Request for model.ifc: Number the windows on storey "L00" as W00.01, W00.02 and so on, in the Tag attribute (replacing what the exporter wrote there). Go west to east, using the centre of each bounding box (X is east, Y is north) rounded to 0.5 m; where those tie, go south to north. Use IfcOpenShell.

First a look at what the model holds.

```python
import ifcopenshell
import ifcopenshell.util.element
import ifcopenshell.util.placement

model = ifcopenshell.open("model.ifc")
print(model.schema)
storey = next(s for s in model.by_type("IfcBuildingStorey") if s.Name == "L00")
windows = [e for e in ifcopenshell.util.element.get_decomposition(storey) if e.is_a("IfcWindow")]
for e in sorted(windows, key=lambda e: e.id()):
    origin = ifcopenshell.util.placement.get_local_placement(e.ObjectPlacement)[:3, 3]
    print(e.id(), e.Tag, e.Name, origin.round(2) + 0.0, sep=" | ")
```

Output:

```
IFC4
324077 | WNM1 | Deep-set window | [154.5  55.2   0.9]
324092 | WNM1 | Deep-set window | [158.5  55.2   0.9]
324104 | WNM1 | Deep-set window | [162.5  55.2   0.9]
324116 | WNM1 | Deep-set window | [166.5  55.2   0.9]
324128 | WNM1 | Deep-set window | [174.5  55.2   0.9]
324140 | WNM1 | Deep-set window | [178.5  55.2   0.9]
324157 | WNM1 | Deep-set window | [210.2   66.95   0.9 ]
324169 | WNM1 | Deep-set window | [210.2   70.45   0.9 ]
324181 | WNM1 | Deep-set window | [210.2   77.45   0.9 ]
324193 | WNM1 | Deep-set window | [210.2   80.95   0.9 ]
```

```python
import ifcopenshell
import ifcopenshell.geom
import ifcopenshell.util.element
import ifcopenshell.util.shape

model = ifcopenshell.open("model.ifc")
settings = ifcopenshell.geom.settings()
settings.set("use-world-coords", True)


def centre(element):
    shape = ifcopenshell.geom.create_shape(settings, element)
    return ifcopenshell.util.shape.get_bbox_centroid(shape.geometry)


storey = next(s for s in model.by_type("IfcBuildingStorey") if s.Name == "L00")
windows = [e for e in ifcopenshell.util.element.get_decomposition(storey) if e.is_a("IfcWindow")]

# Insertion points can sit at a corner or the storey origin, so sort by the geometry (in metres).
centres = {e: centre(e) for e in windows}
windows.sort(key=lambda e: (round(centres[e][0] / 0.5), centres[e][1]))

for i, e in enumerate(windows, start=1):
    number = f"W00.{i:02d}"
    e.Tag = number
    print(e.id(), number)

model.write("model_edited.ifc")
```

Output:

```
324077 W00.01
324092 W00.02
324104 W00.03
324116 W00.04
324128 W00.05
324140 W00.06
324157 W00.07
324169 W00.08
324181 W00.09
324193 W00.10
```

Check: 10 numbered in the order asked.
